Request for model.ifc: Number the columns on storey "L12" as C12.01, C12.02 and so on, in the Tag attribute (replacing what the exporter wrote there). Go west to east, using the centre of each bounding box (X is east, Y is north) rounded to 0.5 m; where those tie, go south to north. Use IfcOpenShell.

First a look at what the model holds.

```python
import ifcopenshell
import ifcopenshell.util.element
import ifcopenshell.util.placement

model = ifcopenshell.open("model.ifc")
print(model.schema)
storey = next(s for s in model.by_type("IfcBuildingStorey") if s.Name == "L12")
columns = [e for e in ifcopenshell.util.element.get_decomposition(storey) if e.is_a("IfcColumn")]
for e in sorted(columns, key=lambda e: e.id()):
    origin = ifcopenshell.util.placement.get_local_placement(e.ObjectPlacement)[:3, 3]
    print(e.id(), e.Tag, e.Name, origin.round(2) + 0.0, sep=" | ")
```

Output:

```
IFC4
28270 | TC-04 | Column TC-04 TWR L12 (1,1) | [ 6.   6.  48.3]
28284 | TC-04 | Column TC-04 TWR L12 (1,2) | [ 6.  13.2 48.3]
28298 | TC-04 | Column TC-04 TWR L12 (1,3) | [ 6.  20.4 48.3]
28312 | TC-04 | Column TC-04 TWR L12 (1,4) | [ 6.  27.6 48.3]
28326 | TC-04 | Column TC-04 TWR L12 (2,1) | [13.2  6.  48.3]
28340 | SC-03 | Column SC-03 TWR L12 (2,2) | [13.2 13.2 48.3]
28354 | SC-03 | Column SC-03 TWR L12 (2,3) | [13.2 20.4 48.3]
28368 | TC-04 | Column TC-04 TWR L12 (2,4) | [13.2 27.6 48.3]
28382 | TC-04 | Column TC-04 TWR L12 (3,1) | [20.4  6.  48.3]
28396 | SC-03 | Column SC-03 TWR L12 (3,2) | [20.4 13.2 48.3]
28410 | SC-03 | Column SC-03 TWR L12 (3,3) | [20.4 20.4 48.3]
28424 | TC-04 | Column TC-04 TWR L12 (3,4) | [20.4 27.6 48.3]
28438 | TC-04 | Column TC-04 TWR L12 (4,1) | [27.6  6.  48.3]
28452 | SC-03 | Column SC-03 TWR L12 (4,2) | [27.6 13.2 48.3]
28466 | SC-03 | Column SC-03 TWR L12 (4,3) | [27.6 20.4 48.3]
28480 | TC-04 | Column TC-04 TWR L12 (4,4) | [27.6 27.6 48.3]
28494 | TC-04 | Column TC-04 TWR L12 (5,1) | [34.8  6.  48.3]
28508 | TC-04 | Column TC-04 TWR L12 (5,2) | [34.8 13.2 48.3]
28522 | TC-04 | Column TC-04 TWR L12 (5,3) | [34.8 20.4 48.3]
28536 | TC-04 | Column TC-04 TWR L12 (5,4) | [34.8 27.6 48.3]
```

```python
import ifcopenshell
import ifcopenshell.geom
import ifcopenshell.util.element
import ifcopenshell.util.shape

model = ifcopenshell.open("model.ifc")
settings = ifcopenshell.geom.settings()
settings.set("use-world-coords", True)


def centre(element):
    shape = ifcopenshell.geom.create_shape(settings, element)
    return ifcopenshell.util.shape.get_bbox_centroid(shape.geometry)


storey = next(s for s in model.by_type("IfcBuildingStorey") if s.Name == "L12")
columns = [e for e in ifcopenshell.util.element.get_decomposition(storey) if e.is_a("IfcColumn")]

# Insertion points can sit at a corner or the storey origin, so sort by the geometry (in metres).
centres = {e: centre(e) for e in columns}
columns.sort(key=lambda e: (round(centres[e][0] / 0.5), centres[e][1]))

for i, e in enumerate(columns, start=1):
    number = f"C12.{i:02d}"
    e.Tag = number
    print(e.id(), number)

model.write("model_edited.ifc")
```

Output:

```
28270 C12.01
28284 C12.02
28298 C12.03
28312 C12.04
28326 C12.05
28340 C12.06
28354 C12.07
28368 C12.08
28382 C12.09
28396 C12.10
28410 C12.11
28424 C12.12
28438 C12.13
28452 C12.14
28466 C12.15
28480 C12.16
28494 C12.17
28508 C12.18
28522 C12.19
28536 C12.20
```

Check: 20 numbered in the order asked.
